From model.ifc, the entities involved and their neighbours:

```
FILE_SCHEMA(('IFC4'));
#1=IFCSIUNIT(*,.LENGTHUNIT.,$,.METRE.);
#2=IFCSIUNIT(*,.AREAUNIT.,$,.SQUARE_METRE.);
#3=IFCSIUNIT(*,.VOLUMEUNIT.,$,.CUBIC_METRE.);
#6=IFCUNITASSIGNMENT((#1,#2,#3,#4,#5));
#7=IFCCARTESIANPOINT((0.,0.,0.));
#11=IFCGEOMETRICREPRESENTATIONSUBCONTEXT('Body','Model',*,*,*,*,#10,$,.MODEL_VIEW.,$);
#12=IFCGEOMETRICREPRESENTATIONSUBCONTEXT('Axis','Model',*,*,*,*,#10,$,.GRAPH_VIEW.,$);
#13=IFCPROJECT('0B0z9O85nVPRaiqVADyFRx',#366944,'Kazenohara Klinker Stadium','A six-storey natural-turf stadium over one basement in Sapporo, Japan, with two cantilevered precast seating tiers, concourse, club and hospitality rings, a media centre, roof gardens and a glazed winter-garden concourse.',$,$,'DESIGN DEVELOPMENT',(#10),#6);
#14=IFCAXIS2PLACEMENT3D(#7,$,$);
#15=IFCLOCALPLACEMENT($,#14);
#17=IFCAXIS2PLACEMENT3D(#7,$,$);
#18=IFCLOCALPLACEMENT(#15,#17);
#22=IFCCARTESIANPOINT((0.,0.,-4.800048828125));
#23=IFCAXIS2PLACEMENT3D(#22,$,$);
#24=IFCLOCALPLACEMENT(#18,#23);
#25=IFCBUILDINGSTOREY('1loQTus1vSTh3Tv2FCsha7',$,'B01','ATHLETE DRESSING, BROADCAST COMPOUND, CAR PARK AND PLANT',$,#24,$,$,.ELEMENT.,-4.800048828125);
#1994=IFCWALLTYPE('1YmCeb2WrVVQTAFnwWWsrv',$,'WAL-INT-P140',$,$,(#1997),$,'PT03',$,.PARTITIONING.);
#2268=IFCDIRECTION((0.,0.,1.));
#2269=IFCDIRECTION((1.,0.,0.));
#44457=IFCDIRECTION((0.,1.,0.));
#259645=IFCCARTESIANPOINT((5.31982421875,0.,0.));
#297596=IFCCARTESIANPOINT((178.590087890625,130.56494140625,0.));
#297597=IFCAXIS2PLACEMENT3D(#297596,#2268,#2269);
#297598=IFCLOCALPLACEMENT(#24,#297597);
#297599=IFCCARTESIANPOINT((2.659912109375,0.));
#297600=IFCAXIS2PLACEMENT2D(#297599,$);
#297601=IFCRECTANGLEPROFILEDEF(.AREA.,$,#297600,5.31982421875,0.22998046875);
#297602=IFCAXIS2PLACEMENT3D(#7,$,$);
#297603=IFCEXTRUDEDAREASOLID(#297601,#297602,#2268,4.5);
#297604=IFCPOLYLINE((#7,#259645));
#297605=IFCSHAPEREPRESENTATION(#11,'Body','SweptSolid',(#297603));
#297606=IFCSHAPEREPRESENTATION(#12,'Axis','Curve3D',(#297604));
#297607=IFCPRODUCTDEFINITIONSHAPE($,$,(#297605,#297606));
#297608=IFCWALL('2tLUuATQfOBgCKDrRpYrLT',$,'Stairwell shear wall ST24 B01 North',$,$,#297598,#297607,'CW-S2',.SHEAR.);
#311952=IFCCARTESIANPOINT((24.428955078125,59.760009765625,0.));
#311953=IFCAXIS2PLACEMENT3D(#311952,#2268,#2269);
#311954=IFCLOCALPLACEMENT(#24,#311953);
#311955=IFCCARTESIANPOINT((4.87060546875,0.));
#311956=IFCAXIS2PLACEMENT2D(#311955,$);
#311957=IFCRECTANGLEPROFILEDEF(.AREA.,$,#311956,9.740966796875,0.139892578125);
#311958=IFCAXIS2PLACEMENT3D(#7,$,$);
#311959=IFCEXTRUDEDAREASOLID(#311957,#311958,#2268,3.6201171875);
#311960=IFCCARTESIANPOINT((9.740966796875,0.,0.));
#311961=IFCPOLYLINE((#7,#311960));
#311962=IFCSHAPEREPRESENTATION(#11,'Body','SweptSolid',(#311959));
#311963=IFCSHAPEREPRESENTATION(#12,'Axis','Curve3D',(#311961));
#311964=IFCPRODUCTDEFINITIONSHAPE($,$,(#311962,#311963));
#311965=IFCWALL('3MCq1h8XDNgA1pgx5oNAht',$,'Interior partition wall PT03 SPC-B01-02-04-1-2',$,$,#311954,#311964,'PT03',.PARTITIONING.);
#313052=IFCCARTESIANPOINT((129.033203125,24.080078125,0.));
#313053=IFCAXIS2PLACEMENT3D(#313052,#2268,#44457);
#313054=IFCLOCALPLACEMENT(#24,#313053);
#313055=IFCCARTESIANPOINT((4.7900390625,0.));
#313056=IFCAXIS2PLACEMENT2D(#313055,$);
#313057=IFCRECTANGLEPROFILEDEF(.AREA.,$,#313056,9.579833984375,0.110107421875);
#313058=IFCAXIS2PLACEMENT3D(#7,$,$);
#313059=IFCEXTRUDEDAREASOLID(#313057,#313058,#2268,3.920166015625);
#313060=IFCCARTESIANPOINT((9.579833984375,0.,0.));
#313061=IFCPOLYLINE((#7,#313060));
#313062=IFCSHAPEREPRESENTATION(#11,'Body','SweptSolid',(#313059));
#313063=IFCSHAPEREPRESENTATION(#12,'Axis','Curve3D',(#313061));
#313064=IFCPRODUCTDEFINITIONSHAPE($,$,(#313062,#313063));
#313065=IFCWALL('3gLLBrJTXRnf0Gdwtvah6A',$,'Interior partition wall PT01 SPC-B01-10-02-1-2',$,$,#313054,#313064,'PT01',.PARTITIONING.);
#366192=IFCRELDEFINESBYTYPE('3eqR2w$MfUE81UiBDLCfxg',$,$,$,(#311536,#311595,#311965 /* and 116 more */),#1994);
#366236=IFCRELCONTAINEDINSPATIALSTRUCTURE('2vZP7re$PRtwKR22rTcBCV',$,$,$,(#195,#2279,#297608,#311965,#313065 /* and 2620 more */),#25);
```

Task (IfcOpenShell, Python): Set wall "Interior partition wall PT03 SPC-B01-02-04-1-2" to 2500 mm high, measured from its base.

```python
import ifcopenshell
import ifcopenshell.geom
import ifcopenshell.util.representation
import ifcopenshell.util.shape

model = ifcopenshell.open("model.ifc")
settings = ifcopenshell.geom.settings()


def volume(element):
    """Net volume in cubic metres, openings subtracted."""
    shape = ifcopenshell.geom.create_shape(settings, element)
    return ifcopenshell.util.shape.get_volume(shape.geometry)


wall = model.by_guid("3MCq1h8XDNgA1pgx5oNAht")
before = volume(wall)

body = ifcopenshell.util.representation.get_representation(wall, "Model", "Body")
solid = body.Items[0]
old_height = solid.Depth
solid.Depth = 2.5
after = volume(wall)

print(f"height {old_height:g} -> {solid.Depth:g}, volume {before:.3f} -> {after:.3f} m3")

model.write("model_edited.ifc")
```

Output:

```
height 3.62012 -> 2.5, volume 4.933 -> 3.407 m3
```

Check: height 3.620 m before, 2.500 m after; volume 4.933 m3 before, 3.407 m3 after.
